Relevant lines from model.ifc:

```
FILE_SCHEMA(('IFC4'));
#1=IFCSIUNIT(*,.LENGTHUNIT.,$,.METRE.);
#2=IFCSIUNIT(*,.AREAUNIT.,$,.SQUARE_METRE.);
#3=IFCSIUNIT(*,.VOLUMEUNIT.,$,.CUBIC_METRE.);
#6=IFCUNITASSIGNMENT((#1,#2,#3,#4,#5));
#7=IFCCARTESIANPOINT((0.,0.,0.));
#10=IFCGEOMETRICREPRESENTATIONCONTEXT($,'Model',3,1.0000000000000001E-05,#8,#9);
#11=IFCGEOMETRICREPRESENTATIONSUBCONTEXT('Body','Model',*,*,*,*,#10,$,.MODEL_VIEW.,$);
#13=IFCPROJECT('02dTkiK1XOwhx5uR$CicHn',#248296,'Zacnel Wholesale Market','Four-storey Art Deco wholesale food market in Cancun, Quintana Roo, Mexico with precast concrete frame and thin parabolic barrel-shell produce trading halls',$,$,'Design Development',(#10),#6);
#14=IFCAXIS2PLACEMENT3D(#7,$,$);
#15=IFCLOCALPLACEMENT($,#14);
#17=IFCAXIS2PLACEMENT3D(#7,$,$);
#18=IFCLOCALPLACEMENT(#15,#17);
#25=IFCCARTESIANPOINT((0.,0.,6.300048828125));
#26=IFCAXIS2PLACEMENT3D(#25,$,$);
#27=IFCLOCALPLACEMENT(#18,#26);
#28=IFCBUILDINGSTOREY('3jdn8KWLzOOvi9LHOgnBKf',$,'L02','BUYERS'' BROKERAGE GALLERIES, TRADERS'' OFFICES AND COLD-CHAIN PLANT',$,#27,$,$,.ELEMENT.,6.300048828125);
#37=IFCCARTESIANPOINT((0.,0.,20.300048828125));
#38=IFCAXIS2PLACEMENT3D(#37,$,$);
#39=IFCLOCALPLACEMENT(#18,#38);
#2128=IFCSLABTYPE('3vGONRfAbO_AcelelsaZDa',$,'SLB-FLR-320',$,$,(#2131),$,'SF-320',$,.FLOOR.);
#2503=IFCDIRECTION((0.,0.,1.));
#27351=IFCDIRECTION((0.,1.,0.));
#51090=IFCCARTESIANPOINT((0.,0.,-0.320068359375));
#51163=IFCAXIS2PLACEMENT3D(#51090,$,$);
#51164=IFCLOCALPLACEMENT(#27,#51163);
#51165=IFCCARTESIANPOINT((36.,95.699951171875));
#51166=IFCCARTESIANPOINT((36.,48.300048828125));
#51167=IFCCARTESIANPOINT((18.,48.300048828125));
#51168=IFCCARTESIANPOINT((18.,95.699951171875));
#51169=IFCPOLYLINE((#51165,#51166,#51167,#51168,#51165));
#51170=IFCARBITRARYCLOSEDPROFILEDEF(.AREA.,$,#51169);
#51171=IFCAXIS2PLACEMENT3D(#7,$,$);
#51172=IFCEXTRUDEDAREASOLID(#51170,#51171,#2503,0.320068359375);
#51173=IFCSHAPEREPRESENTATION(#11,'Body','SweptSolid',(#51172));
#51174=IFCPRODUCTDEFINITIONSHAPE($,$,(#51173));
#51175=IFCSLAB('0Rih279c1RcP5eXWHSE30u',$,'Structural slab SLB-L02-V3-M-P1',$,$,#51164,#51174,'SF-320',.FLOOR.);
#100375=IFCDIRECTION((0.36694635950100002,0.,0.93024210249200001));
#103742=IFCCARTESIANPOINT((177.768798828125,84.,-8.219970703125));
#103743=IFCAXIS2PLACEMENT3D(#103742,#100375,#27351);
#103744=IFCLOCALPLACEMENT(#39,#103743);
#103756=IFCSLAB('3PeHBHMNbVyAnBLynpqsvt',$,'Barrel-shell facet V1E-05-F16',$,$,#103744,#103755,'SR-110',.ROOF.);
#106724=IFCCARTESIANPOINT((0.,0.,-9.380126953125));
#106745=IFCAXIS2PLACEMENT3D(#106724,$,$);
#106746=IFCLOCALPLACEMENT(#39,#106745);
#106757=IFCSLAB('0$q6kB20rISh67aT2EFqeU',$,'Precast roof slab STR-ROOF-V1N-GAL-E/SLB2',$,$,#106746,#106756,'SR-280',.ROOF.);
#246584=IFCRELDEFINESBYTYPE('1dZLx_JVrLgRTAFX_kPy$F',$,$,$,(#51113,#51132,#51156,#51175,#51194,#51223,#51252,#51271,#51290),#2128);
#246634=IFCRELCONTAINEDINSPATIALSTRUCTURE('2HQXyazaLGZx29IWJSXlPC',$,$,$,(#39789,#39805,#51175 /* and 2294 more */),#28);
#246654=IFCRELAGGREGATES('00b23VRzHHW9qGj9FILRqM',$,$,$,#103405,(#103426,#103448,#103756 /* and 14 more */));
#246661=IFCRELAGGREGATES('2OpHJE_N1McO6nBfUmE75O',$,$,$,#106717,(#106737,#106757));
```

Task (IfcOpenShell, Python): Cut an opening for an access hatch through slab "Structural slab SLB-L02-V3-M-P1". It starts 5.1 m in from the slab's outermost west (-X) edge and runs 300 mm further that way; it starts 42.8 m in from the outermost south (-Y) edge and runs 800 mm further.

```python
import numpy as np
import ifcopenshell
import ifcopenshell.api.feature
import ifcopenshell.api.geometry
import ifcopenshell.api.root
import ifcopenshell.geom
import ifcopenshell.util.placement
import ifcopenshell.util.representation
import ifcopenshell.util.shape
import ifcopenshell.util.unit

model = ifcopenshell.open("model.ifc")
unit_scale = ifcopenshell.util.unit.calculate_unit_scale(model)
settings = ifcopenshell.geom.settings()


def volume(element):
    """Net volume in cubic metres, openings subtracted."""
    shape = ifcopenshell.geom.create_shape(settings, element)
    return ifcopenshell.util.shape.get_volume(shape.geometry)


slab = model.by_guid("0Rih279c1RcP5eXWHSE30u")
before = volume(slab)

# Extent in the slab's own axes, in metres. The edges named are its -X and -Y sides.
slab_shape = ifcopenshell.geom.create_shape(settings, slab)
vertices = ifcopenshell.util.shape.get_vertices(slab_shape.geometry)
x_min, y_min, bottom = vertices.min(axis=0)
top = vertices[:, 2].max()

opening = ifcopenshell.api.root.create_entity(model, ifc_class="IfcOpeningElement", name="Access hatch opening", predefined_type="OPENING")
context = ifcopenshell.util.representation.get_context(model, "Model", "Body", "MODEL_VIEW")
width, depth = 0.3, 0.8
outline = [(0.0, 0.0), (width, 0.0), (width, depth), (0.0, depth), (0.0, 0.0)]
# Overshoot both faces by 50 mm so the cut is clean.
shape = ifcopenshell.api.geometry.add_slab_representation(
    model, context=context, depth=top - bottom + 0.1, polyline=outline
)
ifcopenshell.api.geometry.assign_representation(model, product=opening, representation=shape)

matrix = ifcopenshell.util.placement.get_local_placement(slab.ObjectPlacement)
matrix[:, 3] = matrix @ np.append(np.array([x_min + 5.1, y_min + 42.8, bottom - 0.05]) / unit_scale, 1.0)
ifcopenshell.api.geometry.edit_object_placement(model, product=opening, matrix=matrix, is_si=False)
ifcopenshell.api.feature.add_feature(model, feature=opening, element=slab)

after = volume(slab)

print(f"slab volume {before:.3f} -> {after:.3f} m3")

model.write("model_rev.ifc")
```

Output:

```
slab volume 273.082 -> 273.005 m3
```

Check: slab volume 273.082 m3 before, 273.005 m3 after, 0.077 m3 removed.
